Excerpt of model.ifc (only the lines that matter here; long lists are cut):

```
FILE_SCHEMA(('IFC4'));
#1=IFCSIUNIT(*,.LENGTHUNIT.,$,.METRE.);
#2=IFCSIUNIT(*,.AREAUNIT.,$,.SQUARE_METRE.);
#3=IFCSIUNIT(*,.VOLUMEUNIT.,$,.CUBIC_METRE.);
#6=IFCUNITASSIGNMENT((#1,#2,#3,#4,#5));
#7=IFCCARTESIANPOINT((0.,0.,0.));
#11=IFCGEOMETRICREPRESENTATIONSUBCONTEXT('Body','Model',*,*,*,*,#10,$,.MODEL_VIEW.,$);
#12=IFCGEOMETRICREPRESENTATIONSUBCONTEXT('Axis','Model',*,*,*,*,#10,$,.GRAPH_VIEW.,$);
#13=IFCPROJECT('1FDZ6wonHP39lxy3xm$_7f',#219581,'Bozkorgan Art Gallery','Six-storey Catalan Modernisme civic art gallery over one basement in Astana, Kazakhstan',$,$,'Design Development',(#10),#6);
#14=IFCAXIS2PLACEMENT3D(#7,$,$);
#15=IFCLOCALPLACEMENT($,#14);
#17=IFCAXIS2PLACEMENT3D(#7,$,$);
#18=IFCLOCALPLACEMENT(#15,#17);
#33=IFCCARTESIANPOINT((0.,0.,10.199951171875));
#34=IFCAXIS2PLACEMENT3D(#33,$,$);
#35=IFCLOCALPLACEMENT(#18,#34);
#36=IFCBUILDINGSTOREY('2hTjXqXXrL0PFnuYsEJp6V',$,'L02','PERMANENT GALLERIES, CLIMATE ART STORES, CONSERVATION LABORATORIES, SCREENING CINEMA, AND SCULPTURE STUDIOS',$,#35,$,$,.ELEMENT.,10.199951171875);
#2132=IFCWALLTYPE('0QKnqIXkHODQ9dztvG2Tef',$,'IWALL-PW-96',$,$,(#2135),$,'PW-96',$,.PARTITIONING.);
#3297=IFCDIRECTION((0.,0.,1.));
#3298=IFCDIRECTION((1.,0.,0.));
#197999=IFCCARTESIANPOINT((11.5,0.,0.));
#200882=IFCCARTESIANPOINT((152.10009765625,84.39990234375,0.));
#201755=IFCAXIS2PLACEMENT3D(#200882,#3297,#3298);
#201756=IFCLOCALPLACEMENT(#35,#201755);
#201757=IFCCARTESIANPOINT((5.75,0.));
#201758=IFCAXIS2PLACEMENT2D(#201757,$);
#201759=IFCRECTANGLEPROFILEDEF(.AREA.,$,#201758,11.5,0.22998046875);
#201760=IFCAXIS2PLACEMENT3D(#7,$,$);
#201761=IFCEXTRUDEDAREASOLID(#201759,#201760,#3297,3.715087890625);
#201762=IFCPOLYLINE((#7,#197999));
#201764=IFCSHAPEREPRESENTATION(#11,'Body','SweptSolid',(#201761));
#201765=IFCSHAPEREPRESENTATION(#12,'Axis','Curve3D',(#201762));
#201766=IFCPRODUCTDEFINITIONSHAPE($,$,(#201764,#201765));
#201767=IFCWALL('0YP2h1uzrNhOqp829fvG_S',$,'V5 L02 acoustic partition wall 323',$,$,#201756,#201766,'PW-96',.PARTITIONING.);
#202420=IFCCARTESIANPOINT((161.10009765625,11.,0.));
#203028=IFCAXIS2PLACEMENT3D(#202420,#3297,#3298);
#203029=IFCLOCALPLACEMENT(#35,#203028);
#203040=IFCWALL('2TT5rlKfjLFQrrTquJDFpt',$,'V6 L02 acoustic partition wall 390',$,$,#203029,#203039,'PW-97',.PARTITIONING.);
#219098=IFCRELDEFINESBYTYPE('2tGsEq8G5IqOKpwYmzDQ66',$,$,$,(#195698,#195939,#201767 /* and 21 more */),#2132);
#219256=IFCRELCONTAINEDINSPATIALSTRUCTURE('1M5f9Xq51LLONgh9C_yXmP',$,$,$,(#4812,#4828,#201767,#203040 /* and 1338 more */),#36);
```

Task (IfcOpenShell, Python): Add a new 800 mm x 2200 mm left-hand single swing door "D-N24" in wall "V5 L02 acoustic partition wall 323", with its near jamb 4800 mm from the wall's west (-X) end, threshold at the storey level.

```python
import numpy as np
import ifcopenshell
import ifcopenshell.api.feature
import ifcopenshell.api.geometry
import ifcopenshell.api.root
import ifcopenshell.api.spatial
import ifcopenshell.geom
import ifcopenshell.util.element
import ifcopenshell.util.placement
import ifcopenshell.util.representation
import ifcopenshell.util.shape
import ifcopenshell.util.unit

model = ifcopenshell.open("model.ifc")
unit_scale = ifcopenshell.util.unit.calculate_unit_scale(model)
settings = ifcopenshell.geom.settings()


def volume(element):
    """Net volume in cubic metres, openings subtracted."""
    shape = ifcopenshell.geom.create_shape(settings, element)
    return ifcopenshell.util.shape.get_volume(shape.geometry)


wall = model.by_guid("0YP2h1uzrNhOqp829fvG_S")
storey = ifcopenshell.util.element.get_container(wall, ifc_class="IfcBuildingStorey")
context = ifcopenshell.util.representation.get_context(model, "Model", "Body", "MODEL_VIEW")
before = volume(wall)

width, height, from_end, sill = 0.8, 2.2, 4.8, 0.0  # metres

# The wall runs along its own X axis, and the end named is its -X end.
wall_shape = ifcopenshell.geom.create_shape(settings, wall)
x, y, z = ifcopenshell.util.shape.get_vertices(wall_shape.geometry).T
start = x.min() + from_end
face, thickness = float(y.min()), float(y.max() - y.min())
wall_matrix = ifcopenshell.util.placement.get_local_placement(wall.ObjectPlacement)
level = ifcopenshell.util.placement.get_local_placement(storey.ObjectPlacement)[2, 3]


def in_wall(x, y):
    """Placement at x, y metres in the wall's axes, at sill height."""
    matrix = wall_matrix.copy()
    matrix[:, 3] = wall_matrix @ np.array([x / unit_scale, y / unit_scale, 0.0, 1.0])
    matrix[2, 3] = level + sill / unit_scale
    return matrix


# Opening: a box that overshoots both wall faces by 50 mm.
opening = ifcopenshell.api.root.create_entity(model, ifc_class="IfcOpeningElement", predefined_type="OPENING")
box = ifcopenshell.api.geometry.add_wall_representation(
    model, context=context, length=width, height=height, thickness=thickness + 0.1
)
ifcopenshell.api.geometry.assign_representation(model, product=opening, representation=box)
ifcopenshell.api.geometry.edit_object_placement(model, product=opening, matrix=in_wall(start, face - 0.05), is_si=False)
ifcopenshell.api.feature.add_feature(model, feature=opening, element=wall)

door = ifcopenshell.api.root.create_entity(model, ifc_class="IfcDoor", name="D-N24", predefined_type="DOOR")
door.OverallWidth, door.OverallHeight = width / unit_scale, height / unit_scale
door.OperationType = "SINGLE_SWING_LEFT"
body = ifcopenshell.api.geometry.add_door_representation(
    model,
    context=context,
    overall_width=door.OverallWidth,
    overall_height=door.OverallHeight,
    operation_type="SINGLE_SWING_LEFT",
    lining_properties={"LiningDepth": thickness / unit_scale, "ThresholdDepth": thickness / unit_scale},
)
ifcopenshell.api.geometry.assign_representation(model, product=door, representation=body)
ifcopenshell.api.spatial.assign_container(model, products=[door], relating_structure=storey)
ifcopenshell.api.feature.add_filling(model, opening=opening, element=door)

# The lining spans the wall, so the door starts at the wall face.
ifcopenshell.api.geometry.edit_object_placement(model, product=door, matrix=in_wall(start, face), is_si=False)

after = volume(wall)

print(f"wall volume {before:.3f} -> {after:.3f} m3")

model.write("model_rev.ifc")
```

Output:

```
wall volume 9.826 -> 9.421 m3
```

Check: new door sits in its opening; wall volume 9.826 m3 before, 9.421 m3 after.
